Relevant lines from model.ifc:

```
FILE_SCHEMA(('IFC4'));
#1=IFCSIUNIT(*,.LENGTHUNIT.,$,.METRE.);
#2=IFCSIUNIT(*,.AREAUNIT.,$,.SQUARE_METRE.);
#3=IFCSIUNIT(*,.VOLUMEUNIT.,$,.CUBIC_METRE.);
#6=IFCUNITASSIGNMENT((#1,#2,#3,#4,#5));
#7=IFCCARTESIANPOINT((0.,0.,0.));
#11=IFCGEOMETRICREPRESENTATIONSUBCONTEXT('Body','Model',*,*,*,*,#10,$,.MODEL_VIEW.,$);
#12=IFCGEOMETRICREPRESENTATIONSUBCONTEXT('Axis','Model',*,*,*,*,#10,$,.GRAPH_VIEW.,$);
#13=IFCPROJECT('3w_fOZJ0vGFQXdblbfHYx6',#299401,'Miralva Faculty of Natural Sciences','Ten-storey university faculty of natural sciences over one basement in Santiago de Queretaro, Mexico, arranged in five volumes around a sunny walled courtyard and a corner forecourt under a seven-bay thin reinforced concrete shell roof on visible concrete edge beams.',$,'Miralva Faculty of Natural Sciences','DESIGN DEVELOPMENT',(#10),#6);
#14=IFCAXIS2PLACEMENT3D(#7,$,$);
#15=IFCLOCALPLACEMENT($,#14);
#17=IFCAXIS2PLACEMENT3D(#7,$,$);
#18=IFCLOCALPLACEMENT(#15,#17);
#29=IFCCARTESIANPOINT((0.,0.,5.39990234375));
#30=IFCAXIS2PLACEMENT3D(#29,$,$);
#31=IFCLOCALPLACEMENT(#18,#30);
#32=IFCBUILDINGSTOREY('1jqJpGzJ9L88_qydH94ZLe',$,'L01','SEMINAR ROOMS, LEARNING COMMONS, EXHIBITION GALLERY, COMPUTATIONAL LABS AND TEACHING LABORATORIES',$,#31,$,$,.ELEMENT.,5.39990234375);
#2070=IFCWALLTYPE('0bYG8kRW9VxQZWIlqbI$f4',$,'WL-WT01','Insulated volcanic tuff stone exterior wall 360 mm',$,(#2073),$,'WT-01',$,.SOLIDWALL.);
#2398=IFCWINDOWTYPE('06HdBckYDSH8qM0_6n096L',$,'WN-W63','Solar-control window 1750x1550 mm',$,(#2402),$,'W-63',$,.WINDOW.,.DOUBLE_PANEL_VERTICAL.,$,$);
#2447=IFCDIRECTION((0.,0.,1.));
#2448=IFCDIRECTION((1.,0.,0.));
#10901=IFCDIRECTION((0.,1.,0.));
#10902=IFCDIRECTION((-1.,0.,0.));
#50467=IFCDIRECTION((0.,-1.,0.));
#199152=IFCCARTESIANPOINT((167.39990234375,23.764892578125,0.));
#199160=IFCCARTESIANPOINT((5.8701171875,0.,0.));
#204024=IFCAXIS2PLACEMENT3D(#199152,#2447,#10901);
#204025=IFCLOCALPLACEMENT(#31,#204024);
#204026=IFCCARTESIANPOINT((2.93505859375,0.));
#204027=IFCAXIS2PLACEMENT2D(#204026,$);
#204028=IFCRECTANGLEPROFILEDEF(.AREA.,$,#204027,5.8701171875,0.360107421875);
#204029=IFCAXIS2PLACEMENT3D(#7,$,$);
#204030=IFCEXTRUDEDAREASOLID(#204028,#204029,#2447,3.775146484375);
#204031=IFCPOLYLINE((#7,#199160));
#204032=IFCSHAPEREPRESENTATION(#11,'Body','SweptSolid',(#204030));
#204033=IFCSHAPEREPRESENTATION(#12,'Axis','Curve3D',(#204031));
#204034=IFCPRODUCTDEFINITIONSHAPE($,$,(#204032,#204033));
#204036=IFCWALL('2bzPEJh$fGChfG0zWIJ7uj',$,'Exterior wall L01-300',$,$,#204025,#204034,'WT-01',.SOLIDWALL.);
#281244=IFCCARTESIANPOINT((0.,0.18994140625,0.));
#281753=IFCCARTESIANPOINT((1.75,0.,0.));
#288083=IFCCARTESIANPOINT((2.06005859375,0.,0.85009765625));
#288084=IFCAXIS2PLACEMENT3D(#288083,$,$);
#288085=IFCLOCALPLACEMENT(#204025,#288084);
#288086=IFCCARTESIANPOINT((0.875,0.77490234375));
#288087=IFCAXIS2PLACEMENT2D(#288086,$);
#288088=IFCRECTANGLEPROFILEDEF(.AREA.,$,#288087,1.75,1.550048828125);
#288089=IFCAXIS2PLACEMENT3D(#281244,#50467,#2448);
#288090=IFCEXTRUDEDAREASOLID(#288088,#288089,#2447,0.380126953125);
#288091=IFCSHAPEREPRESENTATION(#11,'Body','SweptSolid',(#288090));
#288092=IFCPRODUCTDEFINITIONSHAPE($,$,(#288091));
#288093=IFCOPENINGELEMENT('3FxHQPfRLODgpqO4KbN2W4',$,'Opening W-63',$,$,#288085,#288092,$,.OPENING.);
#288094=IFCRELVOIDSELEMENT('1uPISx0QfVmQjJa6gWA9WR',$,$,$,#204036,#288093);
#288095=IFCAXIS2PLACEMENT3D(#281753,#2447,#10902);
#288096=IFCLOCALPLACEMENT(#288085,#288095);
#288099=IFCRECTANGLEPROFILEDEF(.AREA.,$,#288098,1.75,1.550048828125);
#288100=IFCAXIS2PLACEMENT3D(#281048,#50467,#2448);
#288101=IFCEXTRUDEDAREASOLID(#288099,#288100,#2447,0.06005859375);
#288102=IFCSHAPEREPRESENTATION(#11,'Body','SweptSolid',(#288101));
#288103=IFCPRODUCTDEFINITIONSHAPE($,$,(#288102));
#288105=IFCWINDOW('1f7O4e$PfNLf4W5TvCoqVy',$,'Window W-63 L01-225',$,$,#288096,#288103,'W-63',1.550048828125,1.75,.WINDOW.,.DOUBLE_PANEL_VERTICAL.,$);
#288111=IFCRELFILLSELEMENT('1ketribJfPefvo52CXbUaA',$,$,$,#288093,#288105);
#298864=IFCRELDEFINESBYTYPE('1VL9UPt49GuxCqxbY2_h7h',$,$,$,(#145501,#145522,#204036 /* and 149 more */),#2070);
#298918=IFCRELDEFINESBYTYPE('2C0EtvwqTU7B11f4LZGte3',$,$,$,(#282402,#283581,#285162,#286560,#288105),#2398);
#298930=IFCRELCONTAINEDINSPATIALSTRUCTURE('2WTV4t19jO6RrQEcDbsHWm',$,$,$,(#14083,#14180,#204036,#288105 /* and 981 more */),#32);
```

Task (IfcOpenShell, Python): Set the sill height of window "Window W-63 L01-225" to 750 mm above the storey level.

```python
import numpy as np
import ifcopenshell
import ifcopenshell.api.geometry
import ifcopenshell.geom
import ifcopenshell.util.element
import ifcopenshell.util.placement
import ifcopenshell.util.shape
import ifcopenshell.util.unit

model = ifcopenshell.open("model.ifc")
unit_scale = ifcopenshell.util.unit.calculate_unit_scale(model)

window = model.by_guid("1f7O4e$PfNLf4W5TvCoqVy")
opening = window.FillsVoids[0].RelatingOpeningElement
storey = ifcopenshell.util.element.get_container(window, ifc_class="IfcBuildingStorey")
level = ifcopenshell.util.placement.get_local_placement(storey.ObjectPlacement)[2, 3]

# The opening's origin need not be at the sill, so measure its lowest point.
shape = ifcopenshell.geom.create_shape(ifcopenshell.geom.settings(), opening)
bottom = ifcopenshell.util.shape.get_shape_bottom_elevation(shape, shape.geometry) / unit_scale
dz = level + 0.75 / unit_scale - bottom

shift = np.array([0.0, 0.0, dz])
# The window is placed relative to its opening, so it follows when the opening moves.
matrix = ifcopenshell.util.placement.get_local_placement(opening.ObjectPlacement)
matrix[:3, 3] += shift
ifcopenshell.api.geometry.edit_object_placement(
    model, product=opening, matrix=matrix, is_si=False, should_transform_children=True
)

print(f"moved by {dz * unit_scale:+.3f} m")

model.write("model_edited.ifc")
```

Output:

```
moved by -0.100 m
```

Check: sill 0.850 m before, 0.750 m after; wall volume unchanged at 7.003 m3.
